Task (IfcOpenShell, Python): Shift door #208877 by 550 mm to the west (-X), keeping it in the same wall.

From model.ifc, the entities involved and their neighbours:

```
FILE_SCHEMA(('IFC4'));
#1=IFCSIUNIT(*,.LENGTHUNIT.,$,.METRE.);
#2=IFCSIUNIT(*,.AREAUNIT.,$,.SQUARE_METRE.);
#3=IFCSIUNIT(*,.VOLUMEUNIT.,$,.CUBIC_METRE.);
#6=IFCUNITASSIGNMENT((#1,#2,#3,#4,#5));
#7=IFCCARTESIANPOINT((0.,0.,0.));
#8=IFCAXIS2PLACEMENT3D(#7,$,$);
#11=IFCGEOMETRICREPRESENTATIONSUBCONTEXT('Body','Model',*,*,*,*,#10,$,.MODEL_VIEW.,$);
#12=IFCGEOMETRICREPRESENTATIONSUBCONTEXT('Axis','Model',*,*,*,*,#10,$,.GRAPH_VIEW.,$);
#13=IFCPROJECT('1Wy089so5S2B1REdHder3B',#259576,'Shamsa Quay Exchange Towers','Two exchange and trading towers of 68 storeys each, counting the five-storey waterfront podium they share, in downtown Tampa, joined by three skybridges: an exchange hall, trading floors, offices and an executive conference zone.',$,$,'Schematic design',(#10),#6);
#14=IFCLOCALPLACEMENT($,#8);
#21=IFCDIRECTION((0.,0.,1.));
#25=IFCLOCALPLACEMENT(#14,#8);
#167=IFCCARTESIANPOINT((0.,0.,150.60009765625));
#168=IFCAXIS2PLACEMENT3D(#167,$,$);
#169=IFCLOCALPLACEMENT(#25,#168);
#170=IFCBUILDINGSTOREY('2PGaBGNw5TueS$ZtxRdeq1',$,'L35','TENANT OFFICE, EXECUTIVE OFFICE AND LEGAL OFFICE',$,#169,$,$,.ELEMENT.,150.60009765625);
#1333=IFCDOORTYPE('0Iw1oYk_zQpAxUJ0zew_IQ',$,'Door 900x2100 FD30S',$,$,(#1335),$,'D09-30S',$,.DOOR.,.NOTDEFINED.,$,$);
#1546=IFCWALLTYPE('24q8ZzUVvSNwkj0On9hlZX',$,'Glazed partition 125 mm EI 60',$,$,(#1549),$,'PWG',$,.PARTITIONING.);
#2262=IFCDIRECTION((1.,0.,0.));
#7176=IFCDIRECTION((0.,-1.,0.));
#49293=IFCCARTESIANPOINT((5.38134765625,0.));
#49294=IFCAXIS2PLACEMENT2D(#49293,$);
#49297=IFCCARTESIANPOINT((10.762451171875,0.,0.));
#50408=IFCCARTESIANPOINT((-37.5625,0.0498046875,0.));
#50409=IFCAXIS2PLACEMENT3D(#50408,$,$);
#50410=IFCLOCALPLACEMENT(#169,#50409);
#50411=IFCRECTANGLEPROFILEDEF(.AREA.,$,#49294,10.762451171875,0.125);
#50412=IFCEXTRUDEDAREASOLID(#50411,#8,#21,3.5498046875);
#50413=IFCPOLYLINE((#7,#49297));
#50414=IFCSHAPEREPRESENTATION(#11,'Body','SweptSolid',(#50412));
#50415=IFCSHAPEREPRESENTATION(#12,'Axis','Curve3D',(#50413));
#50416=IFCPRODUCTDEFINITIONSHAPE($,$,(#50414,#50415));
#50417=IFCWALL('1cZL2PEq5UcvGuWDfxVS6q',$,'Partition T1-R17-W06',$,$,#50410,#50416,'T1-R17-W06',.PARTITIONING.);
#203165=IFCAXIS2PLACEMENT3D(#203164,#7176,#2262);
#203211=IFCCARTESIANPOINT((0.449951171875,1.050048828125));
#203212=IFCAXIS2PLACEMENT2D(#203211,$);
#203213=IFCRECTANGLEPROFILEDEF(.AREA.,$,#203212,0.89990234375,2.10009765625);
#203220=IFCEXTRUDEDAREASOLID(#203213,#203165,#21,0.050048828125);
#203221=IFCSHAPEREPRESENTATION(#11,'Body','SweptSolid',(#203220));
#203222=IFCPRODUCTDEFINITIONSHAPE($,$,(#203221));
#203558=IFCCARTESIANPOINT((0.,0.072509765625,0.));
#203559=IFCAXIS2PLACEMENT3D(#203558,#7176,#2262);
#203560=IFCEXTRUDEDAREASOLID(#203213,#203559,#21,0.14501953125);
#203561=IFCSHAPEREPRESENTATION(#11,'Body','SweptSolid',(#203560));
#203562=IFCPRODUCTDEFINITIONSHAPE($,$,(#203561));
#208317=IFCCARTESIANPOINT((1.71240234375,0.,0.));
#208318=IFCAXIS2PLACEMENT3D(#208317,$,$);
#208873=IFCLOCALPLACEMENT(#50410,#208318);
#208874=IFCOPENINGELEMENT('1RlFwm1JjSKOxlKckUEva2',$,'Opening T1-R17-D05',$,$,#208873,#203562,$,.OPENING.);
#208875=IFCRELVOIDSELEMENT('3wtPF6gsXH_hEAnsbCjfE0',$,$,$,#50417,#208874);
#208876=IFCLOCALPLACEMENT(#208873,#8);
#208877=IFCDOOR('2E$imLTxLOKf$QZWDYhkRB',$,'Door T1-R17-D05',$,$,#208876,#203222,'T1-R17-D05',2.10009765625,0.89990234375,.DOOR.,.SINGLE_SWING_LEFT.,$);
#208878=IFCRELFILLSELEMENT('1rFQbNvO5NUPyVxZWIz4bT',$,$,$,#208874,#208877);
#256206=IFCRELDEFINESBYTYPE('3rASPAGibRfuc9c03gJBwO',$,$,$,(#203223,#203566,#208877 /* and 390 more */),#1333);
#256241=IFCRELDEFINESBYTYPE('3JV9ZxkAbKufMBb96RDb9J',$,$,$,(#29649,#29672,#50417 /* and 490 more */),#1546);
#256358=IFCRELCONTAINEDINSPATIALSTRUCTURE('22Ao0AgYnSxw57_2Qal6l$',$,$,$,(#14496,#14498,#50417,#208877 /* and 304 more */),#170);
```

```python
import ifcopenshell
import ifcopenshell.api.geometry
import ifcopenshell.util.placement
import ifcopenshell.util.unit

model = ifcopenshell.open("model.ifc")
unit_scale = ifcopenshell.util.unit.calculate_unit_scale(model)

door = model.by_guid("2E$imLTxLOKf$QZWDYhkRB")
opening = door.FillsVoids[0].RelatingOpeningElement
wall = opening.VoidsElements[0].RelatingBuildingElement

wall_matrix = ifcopenshell.util.placement.get_local_placement(wall.ObjectPlacement)
shift = wall_matrix[:3, 0] * -0.55 / unit_scale
before = ifcopenshell.util.placement.get_local_placement(door.ObjectPlacement)[:3, 3].copy()

# The door is placed relative to its opening, so it follows when the opening moves.
matrix = ifcopenshell.util.placement.get_local_placement(opening.ObjectPlacement)
matrix[:3, 3] += shift
ifcopenshell.api.geometry.edit_object_placement(
    model, product=opening, matrix=matrix, is_si=False, should_transform_children=True
)

after = ifcopenshell.util.placement.get_local_placement(door.ObjectPlacement)[:3, 3]
print("door moved by", (after - before).round(3) + 0.0)

model.write("model_v2.ifc")
```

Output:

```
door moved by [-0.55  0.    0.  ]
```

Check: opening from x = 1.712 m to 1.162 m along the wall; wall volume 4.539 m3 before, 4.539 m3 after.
